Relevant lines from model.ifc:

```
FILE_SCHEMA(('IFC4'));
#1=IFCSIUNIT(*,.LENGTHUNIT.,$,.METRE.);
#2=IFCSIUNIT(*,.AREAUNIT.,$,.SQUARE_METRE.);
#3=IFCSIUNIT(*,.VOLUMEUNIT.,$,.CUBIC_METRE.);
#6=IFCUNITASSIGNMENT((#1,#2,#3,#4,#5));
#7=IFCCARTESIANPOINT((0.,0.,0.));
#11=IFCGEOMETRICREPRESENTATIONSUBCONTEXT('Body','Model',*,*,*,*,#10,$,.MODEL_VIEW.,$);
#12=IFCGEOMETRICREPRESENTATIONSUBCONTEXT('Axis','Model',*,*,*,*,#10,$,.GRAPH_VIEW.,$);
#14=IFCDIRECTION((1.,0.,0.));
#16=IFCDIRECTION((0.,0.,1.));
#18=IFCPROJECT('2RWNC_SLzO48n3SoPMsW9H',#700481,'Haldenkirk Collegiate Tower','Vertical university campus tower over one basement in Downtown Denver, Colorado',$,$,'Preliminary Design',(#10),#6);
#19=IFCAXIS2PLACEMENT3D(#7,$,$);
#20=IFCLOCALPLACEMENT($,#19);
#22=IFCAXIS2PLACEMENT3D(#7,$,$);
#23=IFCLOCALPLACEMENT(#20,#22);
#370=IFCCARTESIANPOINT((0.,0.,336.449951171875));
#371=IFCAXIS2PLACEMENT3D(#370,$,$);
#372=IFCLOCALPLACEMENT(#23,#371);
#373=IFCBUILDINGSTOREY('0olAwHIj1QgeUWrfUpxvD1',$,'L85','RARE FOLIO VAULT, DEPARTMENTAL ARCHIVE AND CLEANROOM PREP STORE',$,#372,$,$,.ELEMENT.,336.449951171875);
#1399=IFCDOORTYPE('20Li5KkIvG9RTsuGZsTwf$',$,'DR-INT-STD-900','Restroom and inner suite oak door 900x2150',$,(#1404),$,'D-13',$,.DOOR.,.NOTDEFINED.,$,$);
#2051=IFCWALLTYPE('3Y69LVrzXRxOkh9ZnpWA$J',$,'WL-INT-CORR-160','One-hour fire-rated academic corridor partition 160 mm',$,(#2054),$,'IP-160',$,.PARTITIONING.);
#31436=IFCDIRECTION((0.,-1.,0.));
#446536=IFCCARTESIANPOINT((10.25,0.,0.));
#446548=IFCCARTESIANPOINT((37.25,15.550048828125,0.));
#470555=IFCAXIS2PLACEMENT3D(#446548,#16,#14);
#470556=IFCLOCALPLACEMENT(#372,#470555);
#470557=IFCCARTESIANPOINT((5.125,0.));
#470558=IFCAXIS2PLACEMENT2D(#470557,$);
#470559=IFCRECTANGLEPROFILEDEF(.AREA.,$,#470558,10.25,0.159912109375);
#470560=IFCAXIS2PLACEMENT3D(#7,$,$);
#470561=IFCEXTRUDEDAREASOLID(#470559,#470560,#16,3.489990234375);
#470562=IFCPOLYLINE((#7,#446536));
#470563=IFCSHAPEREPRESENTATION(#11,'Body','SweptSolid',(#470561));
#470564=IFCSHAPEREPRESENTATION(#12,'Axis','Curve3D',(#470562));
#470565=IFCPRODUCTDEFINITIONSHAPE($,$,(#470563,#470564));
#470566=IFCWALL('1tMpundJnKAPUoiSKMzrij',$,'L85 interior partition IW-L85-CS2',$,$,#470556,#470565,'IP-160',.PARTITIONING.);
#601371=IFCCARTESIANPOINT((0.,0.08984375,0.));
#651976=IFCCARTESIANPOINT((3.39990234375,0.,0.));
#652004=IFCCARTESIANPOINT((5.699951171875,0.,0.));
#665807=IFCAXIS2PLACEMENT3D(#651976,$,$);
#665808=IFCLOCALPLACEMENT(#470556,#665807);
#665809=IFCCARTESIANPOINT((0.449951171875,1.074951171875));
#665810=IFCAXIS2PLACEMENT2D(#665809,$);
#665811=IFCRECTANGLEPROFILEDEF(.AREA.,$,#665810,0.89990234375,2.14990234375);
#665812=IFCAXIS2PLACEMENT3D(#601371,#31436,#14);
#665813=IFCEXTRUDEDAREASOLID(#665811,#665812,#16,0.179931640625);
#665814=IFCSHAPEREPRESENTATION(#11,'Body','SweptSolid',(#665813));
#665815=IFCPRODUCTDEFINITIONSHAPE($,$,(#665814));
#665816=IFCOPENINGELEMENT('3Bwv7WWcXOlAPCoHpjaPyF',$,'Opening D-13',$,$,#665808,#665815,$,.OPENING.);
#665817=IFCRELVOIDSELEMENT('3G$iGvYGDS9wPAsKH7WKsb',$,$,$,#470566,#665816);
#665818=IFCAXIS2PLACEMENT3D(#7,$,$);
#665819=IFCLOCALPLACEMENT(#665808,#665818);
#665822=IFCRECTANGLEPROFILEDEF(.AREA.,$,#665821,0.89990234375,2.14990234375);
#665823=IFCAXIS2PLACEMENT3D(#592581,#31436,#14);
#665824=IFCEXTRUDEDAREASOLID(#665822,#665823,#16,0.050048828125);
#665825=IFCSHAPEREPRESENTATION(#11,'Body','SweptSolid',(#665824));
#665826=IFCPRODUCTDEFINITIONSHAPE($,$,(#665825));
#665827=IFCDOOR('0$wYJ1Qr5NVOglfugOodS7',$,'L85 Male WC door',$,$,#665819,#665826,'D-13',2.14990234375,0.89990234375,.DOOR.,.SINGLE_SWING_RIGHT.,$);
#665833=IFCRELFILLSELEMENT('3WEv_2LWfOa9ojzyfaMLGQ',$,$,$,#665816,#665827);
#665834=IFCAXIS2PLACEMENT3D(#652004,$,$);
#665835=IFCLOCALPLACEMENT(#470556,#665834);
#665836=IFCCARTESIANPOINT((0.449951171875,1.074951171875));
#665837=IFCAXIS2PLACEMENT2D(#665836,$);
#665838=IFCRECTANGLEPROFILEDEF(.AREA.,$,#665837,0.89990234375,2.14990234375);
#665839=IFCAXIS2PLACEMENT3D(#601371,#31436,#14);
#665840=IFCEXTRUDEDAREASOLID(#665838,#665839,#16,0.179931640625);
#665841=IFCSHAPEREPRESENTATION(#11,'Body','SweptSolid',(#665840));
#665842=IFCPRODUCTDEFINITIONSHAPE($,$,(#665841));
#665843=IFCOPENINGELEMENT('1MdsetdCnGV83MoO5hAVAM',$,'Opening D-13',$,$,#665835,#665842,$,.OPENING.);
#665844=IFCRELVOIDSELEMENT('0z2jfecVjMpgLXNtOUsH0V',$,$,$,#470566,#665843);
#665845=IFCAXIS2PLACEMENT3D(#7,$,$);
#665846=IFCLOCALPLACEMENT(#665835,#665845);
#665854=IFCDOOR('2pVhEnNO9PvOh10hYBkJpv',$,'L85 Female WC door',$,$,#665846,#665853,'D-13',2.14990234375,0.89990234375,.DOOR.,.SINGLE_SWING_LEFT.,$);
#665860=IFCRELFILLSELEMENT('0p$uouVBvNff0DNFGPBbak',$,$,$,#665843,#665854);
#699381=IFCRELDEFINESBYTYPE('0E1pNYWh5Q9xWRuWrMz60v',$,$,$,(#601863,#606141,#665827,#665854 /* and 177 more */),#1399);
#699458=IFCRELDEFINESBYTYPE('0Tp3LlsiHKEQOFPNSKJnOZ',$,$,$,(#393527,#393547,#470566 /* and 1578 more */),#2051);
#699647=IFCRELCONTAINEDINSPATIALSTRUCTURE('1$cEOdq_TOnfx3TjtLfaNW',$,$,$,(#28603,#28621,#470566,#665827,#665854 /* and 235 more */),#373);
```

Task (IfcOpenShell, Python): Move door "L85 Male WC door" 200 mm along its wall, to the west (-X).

```python
import ifcopenshell
import ifcopenshell.api.geometry
import ifcopenshell.util.placement
import ifcopenshell.util.unit

model = ifcopenshell.open("model.ifc")
unit_scale = ifcopenshell.util.unit.calculate_unit_scale(model)

door = model.by_guid("0$wYJ1Qr5NVOglfugOodS7")
opening = door.FillsVoids[0].RelatingOpeningElement
wall = opening.VoidsElements[0].RelatingBuildingElement

wall_matrix = ifcopenshell.util.placement.get_local_placement(wall.ObjectPlacement)
shift = wall_matrix[:3, 0] * -0.2 / unit_scale
before = ifcopenshell.util.placement.get_local_placement(door.ObjectPlacement)[:3, 3].copy()

# The door is placed relative to its opening, so it follows when the opening moves.
matrix = ifcopenshell.util.placement.get_local_placement(opening.ObjectPlacement)
matrix[:3, 3] += shift
ifcopenshell.api.geometry.edit_object_placement(
    model, product=opening, matrix=matrix, is_si=False, should_transform_children=True
)

after = ifcopenshell.util.placement.get_local_placement(door.ObjectPlacement)[:3, 3]
print("door moved by", (after - before).round(3) + 0.0)

model.write("model_edited.ifc")
```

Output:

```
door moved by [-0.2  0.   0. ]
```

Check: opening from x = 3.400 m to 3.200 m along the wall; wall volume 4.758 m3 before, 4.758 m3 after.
